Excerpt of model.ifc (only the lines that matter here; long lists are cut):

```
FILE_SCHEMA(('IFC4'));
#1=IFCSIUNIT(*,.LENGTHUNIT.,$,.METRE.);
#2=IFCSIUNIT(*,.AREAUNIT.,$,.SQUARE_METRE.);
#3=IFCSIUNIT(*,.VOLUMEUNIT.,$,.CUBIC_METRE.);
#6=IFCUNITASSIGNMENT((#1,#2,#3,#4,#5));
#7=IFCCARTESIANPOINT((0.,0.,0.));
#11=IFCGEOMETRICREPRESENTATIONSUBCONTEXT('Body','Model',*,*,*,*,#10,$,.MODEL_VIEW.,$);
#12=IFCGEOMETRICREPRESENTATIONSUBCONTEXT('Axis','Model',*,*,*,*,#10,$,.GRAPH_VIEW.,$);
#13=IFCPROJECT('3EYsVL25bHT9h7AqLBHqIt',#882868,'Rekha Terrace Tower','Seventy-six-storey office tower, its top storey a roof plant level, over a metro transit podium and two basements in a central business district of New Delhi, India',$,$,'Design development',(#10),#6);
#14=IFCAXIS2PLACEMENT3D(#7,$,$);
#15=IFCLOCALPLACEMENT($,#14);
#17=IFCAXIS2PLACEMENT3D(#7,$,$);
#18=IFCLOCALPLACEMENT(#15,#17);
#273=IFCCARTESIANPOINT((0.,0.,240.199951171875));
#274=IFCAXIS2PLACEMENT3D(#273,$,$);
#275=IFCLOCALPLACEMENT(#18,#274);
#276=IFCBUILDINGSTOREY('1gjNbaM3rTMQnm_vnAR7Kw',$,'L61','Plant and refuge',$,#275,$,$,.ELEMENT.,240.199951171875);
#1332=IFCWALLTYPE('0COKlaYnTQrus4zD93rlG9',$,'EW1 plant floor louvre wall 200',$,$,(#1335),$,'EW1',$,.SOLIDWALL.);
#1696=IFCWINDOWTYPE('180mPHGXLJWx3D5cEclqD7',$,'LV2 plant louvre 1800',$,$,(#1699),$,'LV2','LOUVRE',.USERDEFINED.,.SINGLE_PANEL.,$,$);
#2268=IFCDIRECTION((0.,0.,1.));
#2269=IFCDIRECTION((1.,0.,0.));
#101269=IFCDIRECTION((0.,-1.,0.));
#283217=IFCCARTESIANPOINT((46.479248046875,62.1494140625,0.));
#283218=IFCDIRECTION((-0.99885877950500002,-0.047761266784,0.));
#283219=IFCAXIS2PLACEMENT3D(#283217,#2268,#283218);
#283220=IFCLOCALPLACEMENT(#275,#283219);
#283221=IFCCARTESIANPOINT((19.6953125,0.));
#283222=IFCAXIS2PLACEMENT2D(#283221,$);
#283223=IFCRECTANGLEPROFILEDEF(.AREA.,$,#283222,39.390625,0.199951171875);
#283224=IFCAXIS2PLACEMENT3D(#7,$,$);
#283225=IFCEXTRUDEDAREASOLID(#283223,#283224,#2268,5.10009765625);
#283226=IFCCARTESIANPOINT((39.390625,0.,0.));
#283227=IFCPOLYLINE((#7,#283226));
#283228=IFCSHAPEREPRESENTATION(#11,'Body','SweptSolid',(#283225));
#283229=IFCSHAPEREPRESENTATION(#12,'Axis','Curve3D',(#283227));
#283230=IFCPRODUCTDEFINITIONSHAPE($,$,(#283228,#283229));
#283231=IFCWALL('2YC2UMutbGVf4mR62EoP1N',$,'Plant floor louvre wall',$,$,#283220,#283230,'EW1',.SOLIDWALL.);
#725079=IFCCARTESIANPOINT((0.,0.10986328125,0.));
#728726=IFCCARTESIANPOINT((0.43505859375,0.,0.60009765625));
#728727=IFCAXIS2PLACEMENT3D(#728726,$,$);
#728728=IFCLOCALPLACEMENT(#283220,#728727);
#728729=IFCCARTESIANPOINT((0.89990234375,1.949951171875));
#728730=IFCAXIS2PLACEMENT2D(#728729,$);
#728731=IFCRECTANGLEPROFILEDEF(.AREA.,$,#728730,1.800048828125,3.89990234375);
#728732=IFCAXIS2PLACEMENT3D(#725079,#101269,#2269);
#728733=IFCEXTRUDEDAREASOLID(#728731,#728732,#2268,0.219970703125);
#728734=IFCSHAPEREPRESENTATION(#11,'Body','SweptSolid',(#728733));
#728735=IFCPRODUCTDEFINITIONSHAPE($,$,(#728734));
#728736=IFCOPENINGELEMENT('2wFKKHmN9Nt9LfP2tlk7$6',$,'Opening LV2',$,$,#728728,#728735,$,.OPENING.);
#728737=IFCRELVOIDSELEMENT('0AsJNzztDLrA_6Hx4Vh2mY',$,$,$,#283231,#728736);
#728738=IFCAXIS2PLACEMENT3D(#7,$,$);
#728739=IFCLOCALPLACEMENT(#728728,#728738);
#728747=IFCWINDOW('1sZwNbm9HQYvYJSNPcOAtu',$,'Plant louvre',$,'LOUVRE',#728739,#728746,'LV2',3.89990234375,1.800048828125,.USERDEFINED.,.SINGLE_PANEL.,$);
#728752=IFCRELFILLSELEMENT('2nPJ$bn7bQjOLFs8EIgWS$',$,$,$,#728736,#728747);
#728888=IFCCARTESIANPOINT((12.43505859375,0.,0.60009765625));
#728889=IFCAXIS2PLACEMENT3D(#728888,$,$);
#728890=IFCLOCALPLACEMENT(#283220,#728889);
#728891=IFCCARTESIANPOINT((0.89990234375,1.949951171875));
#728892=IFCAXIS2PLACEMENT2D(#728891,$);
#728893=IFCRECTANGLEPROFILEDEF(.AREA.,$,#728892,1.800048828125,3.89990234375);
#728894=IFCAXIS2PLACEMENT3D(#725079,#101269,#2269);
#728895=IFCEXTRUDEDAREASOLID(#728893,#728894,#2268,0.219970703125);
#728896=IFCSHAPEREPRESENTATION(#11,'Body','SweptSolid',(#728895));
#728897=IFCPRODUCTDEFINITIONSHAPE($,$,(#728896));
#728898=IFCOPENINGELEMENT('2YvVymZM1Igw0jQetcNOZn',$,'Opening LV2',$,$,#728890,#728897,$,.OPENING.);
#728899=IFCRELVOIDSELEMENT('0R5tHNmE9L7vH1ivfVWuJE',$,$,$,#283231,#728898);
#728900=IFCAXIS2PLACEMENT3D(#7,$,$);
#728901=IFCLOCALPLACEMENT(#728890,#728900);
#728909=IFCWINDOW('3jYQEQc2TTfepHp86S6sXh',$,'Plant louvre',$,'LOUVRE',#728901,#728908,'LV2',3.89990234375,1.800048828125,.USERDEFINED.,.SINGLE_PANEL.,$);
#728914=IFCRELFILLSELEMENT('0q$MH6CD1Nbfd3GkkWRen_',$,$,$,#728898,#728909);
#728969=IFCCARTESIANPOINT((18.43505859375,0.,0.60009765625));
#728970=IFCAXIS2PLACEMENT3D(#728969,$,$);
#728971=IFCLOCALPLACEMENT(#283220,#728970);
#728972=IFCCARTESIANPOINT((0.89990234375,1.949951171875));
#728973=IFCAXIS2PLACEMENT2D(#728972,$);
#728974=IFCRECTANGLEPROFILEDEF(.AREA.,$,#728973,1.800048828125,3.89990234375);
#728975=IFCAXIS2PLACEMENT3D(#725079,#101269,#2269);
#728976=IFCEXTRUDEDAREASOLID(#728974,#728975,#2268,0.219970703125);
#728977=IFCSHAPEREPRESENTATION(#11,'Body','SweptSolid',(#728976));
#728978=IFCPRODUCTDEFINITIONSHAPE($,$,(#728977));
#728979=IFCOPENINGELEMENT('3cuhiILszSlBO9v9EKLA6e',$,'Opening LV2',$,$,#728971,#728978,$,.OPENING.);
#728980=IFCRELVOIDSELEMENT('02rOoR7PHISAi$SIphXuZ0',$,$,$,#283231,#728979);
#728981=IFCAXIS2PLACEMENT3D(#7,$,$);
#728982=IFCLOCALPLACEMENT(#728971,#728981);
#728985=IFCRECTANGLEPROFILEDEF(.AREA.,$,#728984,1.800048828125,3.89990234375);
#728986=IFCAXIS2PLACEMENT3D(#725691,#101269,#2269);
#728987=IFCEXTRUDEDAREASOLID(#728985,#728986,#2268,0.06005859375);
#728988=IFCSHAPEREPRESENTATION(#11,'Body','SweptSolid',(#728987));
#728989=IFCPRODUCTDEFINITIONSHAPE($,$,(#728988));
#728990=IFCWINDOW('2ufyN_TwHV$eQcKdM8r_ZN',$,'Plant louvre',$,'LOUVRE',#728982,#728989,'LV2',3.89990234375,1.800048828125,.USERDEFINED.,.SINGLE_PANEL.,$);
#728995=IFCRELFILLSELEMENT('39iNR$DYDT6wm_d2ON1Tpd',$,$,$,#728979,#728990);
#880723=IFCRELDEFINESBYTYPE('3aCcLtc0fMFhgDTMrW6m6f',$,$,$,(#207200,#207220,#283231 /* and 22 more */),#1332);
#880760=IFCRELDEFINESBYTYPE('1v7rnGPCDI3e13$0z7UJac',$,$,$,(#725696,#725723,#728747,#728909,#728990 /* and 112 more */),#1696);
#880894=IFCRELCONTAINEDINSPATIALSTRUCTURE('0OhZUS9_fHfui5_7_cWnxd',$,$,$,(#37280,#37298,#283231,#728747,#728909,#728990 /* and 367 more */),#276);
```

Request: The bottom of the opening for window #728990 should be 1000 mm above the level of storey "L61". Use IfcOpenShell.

```python
import numpy as np
import ifcopenshell
import ifcopenshell.api.geometry
import ifcopenshell.geom
import ifcopenshell.util.element
import ifcopenshell.util.placement
import ifcopenshell.util.shape
import ifcopenshell.util.unit

model = ifcopenshell.open("model.ifc")
unit_scale = ifcopenshell.util.unit.calculate_unit_scale(model)

window = model.by_guid("2ufyN_TwHV$eQcKdM8r_ZN")
opening = window.FillsVoids[0].RelatingOpeningElement
storey = ifcopenshell.util.element.get_container(window, ifc_class="IfcBuildingStorey")
level = ifcopenshell.util.placement.get_local_placement(storey.ObjectPlacement)[2, 3]

# The opening's origin need not be at the sill, so measure its lowest point.
shape = ifcopenshell.geom.create_shape(ifcopenshell.geom.settings(), opening)
bottom = ifcopenshell.util.shape.get_shape_bottom_elevation(shape, shape.geometry) / unit_scale
dz = level + 1 / unit_scale - bottom

shift = np.array([0.0, 0.0, dz])
# The window is placed relative to its opening, so it follows when the opening moves.
matrix = ifcopenshell.util.placement.get_local_placement(opening.ObjectPlacement)
matrix[:3, 3] += shift
ifcopenshell.api.geometry.edit_object_placement(
    model, product=opening, matrix=matrix, is_si=False, should_transform_children=True
)

print(f"moved by {dz * unit_scale:+.3f} m")

model.write("model_v2.ifc")
```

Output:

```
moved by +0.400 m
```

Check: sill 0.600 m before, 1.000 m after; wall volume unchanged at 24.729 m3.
